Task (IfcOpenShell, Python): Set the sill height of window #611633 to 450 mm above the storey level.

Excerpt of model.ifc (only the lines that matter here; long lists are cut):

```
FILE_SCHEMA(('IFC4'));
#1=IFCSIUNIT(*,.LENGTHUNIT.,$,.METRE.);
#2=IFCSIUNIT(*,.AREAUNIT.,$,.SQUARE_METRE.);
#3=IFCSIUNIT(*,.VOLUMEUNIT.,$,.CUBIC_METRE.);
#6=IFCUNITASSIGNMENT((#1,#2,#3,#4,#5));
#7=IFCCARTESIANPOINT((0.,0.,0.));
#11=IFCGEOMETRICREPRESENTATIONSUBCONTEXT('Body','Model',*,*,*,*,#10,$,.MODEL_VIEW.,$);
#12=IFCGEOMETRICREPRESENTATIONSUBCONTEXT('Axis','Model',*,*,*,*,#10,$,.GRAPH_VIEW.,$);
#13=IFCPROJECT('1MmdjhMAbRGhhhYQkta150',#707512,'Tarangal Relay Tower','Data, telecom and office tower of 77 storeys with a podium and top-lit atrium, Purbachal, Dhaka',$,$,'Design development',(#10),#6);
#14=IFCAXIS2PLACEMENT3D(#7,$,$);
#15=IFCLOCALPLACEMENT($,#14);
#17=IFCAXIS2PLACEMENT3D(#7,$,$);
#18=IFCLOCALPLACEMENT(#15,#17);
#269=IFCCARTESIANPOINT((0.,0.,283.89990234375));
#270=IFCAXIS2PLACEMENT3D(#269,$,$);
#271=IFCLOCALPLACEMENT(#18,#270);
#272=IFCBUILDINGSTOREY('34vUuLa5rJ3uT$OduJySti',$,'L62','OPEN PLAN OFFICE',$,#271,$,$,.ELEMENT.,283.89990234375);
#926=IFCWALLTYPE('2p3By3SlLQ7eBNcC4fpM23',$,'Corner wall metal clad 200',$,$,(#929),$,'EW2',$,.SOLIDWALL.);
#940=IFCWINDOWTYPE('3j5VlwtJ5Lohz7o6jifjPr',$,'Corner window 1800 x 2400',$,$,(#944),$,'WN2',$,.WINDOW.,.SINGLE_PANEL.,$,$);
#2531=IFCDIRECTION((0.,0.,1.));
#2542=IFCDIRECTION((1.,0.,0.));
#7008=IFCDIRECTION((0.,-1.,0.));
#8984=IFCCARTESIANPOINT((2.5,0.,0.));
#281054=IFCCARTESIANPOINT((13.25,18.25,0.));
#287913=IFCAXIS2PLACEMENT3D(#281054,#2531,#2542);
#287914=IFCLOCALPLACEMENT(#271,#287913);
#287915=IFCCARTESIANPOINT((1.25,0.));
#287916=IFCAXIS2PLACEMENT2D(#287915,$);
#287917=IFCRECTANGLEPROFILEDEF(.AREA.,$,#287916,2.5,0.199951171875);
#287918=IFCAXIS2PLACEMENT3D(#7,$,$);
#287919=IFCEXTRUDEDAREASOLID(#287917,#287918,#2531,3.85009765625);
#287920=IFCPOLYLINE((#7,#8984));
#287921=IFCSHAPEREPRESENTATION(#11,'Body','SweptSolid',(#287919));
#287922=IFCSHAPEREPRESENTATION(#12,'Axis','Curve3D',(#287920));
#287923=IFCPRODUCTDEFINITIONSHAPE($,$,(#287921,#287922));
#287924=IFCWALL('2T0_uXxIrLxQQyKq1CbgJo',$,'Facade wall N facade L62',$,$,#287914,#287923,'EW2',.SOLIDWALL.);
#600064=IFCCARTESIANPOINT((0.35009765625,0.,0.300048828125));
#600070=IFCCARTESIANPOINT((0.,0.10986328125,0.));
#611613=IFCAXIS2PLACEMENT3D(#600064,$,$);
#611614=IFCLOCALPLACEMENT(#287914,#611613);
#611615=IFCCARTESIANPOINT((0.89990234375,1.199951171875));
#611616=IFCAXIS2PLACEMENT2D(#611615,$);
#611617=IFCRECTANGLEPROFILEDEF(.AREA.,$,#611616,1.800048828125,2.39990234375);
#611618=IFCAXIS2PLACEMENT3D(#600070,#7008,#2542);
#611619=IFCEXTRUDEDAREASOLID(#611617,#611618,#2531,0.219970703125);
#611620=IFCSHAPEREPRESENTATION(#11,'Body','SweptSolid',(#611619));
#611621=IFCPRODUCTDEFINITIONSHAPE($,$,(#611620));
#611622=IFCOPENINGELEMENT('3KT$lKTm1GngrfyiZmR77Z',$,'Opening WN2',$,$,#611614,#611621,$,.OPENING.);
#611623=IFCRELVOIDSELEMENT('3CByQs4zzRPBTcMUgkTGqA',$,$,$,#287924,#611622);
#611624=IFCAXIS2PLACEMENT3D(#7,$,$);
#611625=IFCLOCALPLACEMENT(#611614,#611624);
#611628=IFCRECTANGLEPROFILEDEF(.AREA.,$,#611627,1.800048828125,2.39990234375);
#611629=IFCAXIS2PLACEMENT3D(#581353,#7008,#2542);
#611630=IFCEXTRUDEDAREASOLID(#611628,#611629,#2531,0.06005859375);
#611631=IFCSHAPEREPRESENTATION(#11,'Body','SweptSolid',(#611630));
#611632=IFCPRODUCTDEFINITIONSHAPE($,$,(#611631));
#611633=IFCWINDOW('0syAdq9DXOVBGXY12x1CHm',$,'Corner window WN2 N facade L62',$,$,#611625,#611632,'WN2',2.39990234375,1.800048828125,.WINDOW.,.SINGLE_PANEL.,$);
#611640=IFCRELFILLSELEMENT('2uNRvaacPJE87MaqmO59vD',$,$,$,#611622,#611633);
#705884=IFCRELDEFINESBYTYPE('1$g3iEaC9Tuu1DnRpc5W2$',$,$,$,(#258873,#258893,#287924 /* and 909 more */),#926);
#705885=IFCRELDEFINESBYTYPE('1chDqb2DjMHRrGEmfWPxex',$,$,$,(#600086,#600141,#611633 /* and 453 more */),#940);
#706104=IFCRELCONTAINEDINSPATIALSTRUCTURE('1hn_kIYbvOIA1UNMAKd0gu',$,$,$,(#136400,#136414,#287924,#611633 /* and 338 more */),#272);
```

```python
import numpy as np
import ifcopenshell
import ifcopenshell.api.geometry
import ifcopenshell.geom
import ifcopenshell.util.element
import ifcopenshell.util.placement
import ifcopenshell.util.shape
import ifcopenshell.util.unit

model = ifcopenshell.open("model.ifc")
unit_scale = ifcopenshell.util.unit.calculate_unit_scale(model)

window = model.by_id(611633)
opening = window.FillsVoids[0].RelatingOpeningElement
storey = ifcopenshell.util.element.get_container(window, ifc_class="IfcBuildingStorey")
level = ifcopenshell.util.placement.get_local_placement(storey.ObjectPlacement)[2, 3]

# The opening's origin need not be at the sill, so measure its lowest point.
shape = ifcopenshell.geom.create_shape(ifcopenshell.geom.settings(), opening)
bottom = ifcopenshell.util.shape.get_shape_bottom_elevation(shape, shape.geometry) / unit_scale
dz = level + 0.45 / unit_scale - bottom

shift = np.array([0.0, 0.0, dz])
# The window is placed relative to its opening, so it follows when the opening moves.
matrix = ifcopenshell.util.placement.get_local_placement(opening.ObjectPlacement)
matrix[:3, 3] += shift
ifcopenshell.api.geometry.edit_object_placement(
    model, product=opening, matrix=matrix, is_si=False, should_transform_children=True
)

print(f"moved by {dz * unit_scale:+.3f} m")

model.write("model-out.ifc")
```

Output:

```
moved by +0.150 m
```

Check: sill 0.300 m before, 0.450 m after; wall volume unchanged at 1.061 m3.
